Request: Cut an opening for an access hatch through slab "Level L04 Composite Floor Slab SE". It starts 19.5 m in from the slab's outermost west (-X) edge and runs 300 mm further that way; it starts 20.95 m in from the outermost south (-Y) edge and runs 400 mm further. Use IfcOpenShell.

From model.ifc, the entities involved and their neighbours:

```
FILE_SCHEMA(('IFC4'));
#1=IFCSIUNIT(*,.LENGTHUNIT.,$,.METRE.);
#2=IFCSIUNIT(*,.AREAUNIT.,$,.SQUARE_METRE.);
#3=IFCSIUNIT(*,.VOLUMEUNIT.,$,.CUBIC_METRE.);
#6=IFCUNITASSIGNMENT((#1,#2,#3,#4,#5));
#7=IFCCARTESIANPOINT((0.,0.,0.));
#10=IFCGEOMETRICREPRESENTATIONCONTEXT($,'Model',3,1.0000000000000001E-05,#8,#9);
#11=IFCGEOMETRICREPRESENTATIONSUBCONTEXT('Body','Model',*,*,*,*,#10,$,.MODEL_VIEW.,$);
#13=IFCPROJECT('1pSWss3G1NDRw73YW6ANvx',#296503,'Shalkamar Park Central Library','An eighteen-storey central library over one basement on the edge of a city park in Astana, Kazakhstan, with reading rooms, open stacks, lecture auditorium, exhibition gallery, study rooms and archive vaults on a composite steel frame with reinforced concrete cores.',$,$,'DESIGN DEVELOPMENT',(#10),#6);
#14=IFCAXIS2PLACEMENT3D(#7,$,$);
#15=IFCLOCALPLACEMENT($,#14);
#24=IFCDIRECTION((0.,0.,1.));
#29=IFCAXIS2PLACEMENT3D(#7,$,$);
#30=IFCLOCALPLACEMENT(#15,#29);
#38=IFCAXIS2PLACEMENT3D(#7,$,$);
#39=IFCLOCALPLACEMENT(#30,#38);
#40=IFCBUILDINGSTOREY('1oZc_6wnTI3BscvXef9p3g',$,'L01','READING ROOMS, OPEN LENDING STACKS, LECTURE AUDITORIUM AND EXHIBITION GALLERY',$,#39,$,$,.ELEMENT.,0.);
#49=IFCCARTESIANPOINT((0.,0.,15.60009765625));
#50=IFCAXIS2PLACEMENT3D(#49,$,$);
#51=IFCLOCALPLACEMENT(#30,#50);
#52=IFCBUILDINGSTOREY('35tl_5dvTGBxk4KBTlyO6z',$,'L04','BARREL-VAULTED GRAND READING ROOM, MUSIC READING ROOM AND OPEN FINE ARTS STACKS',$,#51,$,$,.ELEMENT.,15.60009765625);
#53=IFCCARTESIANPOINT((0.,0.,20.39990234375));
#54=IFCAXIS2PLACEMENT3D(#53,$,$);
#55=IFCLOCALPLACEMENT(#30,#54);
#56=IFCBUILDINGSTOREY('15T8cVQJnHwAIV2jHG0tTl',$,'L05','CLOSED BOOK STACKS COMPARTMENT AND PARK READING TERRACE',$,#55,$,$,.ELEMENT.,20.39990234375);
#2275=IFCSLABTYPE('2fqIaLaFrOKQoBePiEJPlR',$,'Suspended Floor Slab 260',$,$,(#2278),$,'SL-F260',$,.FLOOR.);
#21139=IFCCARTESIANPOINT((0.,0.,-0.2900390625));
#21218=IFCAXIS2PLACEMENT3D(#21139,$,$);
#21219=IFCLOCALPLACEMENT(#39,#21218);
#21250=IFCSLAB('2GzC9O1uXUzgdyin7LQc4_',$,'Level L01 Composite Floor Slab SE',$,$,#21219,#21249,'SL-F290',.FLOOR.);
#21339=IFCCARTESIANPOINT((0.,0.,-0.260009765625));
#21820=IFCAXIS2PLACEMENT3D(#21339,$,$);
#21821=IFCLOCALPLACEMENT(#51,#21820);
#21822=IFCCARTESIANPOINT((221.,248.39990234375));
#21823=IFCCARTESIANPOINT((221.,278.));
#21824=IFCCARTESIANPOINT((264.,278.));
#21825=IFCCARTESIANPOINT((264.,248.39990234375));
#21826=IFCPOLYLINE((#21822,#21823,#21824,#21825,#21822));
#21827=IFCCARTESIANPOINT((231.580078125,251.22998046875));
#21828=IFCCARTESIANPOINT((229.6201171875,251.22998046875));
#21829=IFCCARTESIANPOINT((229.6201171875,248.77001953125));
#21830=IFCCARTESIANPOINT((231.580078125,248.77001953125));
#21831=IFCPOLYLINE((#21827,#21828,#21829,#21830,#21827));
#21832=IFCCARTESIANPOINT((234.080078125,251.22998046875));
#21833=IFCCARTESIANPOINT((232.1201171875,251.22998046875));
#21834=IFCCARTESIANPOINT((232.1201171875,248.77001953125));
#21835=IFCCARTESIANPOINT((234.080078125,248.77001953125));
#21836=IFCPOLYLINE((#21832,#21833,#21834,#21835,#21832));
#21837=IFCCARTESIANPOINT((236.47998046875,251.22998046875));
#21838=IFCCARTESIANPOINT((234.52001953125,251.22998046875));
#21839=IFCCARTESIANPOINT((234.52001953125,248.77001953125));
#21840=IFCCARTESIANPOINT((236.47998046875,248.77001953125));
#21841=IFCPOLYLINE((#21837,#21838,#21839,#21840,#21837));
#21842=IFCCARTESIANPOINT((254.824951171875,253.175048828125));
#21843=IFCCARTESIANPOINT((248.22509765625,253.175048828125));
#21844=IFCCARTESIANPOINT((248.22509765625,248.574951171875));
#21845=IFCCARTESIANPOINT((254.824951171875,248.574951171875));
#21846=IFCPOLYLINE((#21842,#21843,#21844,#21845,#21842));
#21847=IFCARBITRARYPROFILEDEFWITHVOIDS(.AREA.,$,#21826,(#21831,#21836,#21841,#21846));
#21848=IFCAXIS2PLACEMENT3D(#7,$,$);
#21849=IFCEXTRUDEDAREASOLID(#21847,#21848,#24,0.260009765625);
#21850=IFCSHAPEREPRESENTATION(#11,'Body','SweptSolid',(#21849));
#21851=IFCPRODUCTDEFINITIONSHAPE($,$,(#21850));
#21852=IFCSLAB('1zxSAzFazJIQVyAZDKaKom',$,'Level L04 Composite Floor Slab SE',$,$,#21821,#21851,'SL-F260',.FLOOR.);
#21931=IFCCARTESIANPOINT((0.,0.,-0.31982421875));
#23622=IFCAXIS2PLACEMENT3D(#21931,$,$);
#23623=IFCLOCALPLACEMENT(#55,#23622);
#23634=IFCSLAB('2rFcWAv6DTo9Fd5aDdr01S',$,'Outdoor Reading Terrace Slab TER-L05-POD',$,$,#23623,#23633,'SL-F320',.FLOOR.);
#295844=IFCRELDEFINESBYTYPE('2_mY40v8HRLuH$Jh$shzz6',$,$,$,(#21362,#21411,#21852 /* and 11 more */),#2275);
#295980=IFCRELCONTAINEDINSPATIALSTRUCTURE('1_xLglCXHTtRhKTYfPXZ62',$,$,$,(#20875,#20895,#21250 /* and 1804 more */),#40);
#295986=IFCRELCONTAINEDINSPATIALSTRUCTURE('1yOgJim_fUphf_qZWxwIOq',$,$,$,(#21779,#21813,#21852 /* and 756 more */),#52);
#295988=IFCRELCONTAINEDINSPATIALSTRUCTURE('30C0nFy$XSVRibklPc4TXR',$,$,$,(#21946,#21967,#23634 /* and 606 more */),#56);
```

```python
import numpy as np
import ifcopenshell
import ifcopenshell.api.feature
import ifcopenshell.api.geometry
import ifcopenshell.api.root
import ifcopenshell.geom
import ifcopenshell.util.placement
import ifcopenshell.util.representation
import ifcopenshell.util.shape
import ifcopenshell.util.unit

model = ifcopenshell.open("model.ifc")
unit_scale = ifcopenshell.util.unit.calculate_unit_scale(model)
settings = ifcopenshell.geom.settings()


def volume(element):
    """Net volume in cubic metres, openings subtracted."""
    shape = ifcopenshell.geom.create_shape(settings, element)
    return ifcopenshell.util.shape.get_volume(shape.geometry)


slab = model.by_guid("1zxSAzFazJIQVyAZDKaKom")
before = volume(slab)

# Extent in the slab's own axes, in metres. The edges named are its -X and -Y sides.
slab_shape = ifcopenshell.geom.create_shape(settings, slab)
vertices = ifcopenshell.util.shape.get_vertices(slab_shape.geometry)
x_min, y_min, bottom = vertices.min(axis=0)
top = vertices[:, 2].max()

opening = ifcopenshell.api.root.create_entity(model, ifc_class="IfcOpeningElement", name="Access hatch opening", predefined_type="OPENING")
context = ifcopenshell.util.representation.get_context(model, "Model", "Body", "MODEL_VIEW")
width, depth = 0.3, 0.4
outline = [(0.0, 0.0), (width, 0.0), (width, depth), (0.0, depth), (0.0, 0.0)]
# Overshoot both faces by 50 mm so the cut is clean.
shape = ifcopenshell.api.geometry.add_slab_representation(
    model, context=context, depth=top - bottom + 0.1, polyline=outline
)
ifcopenshell.api.geometry.assign_representation(model, product=opening, representation=shape)

matrix = ifcopenshell.util.placement.get_local_placement(slab.ObjectPlacement)
matrix[:, 3] = matrix @ np.append(np.array([x_min + 19.5, y_min + 20.95, bottom - 0.05]) / unit_scale, 1.0)
ifcopenshell.api.geometry.edit_object_placement(model, product=opening, matrix=matrix, is_si=False)
ifcopenshell.api.feature.add_feature(model, feature=opening, element=slab)

after = volume(slab)

print(f"slab volume {before:.3f} -> {after:.3f} m3")

model.write("model_v2.ifc")
```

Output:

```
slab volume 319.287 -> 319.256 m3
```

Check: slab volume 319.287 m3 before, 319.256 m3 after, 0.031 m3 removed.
